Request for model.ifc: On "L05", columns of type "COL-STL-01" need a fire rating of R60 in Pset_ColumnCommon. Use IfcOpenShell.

First a look at what the model holds.

```python
import ifcopenshell
import ifcopenshell.util.element

model = ifcopenshell.open("model.ifc")
print(model.schema)
storey = next(s for s in model.by_type("IfcBuildingStorey") if s.Name == "L05")
columns = [e for e in ifcopenshell.util.element.get_decomposition(storey) if e.is_a("IfcColumn")]
seen = {}
for e in columns:
    element_type = ifcopenshell.util.element.get_type(e)
    key = (element_type.Name if element_type != e and element_type else None, ifcopenshell.util.element.get_pset(e, "Pset_ColumnCommon", "FireRating"))
    seen[key] = seen.get(key, 0) + 1
for (name, value), count in sorted(seen.items(), key=str):
    print(count, "x", name, "|", value)
```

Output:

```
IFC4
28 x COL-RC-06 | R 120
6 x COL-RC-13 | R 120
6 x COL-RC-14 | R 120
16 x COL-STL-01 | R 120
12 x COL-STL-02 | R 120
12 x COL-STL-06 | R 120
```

```python
import ifcopenshell
import ifcopenshell.api.pset
import ifcopenshell.util.element

model = ifcopenshell.open("model.ifc")

storey = next(s for s in model.by_type("IfcBuildingStorey") if s.Name == "L05")
columns = [e for e in ifcopenshell.util.element.get_decomposition(storey) if e.is_a("IfcColumn")]

count = 0
for e in columns:
    element_type = ifcopenshell.util.element.get_type(e)
    if element_type in (None, e) or element_type.Name != "COL-STL-01":
        continue
    # add_pset returns the element's existing set when there is one.
    pset = ifcopenshell.api.pset.add_pset(model, product=e, name="Pset_ColumnCommon")
    ifcopenshell.api.pset.edit_pset(model, pset=pset, properties={"FireRating": "R60"})
    count += 1

print(count, "columns updated")

model.write("model_v2.ifc")
```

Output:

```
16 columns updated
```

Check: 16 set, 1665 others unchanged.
